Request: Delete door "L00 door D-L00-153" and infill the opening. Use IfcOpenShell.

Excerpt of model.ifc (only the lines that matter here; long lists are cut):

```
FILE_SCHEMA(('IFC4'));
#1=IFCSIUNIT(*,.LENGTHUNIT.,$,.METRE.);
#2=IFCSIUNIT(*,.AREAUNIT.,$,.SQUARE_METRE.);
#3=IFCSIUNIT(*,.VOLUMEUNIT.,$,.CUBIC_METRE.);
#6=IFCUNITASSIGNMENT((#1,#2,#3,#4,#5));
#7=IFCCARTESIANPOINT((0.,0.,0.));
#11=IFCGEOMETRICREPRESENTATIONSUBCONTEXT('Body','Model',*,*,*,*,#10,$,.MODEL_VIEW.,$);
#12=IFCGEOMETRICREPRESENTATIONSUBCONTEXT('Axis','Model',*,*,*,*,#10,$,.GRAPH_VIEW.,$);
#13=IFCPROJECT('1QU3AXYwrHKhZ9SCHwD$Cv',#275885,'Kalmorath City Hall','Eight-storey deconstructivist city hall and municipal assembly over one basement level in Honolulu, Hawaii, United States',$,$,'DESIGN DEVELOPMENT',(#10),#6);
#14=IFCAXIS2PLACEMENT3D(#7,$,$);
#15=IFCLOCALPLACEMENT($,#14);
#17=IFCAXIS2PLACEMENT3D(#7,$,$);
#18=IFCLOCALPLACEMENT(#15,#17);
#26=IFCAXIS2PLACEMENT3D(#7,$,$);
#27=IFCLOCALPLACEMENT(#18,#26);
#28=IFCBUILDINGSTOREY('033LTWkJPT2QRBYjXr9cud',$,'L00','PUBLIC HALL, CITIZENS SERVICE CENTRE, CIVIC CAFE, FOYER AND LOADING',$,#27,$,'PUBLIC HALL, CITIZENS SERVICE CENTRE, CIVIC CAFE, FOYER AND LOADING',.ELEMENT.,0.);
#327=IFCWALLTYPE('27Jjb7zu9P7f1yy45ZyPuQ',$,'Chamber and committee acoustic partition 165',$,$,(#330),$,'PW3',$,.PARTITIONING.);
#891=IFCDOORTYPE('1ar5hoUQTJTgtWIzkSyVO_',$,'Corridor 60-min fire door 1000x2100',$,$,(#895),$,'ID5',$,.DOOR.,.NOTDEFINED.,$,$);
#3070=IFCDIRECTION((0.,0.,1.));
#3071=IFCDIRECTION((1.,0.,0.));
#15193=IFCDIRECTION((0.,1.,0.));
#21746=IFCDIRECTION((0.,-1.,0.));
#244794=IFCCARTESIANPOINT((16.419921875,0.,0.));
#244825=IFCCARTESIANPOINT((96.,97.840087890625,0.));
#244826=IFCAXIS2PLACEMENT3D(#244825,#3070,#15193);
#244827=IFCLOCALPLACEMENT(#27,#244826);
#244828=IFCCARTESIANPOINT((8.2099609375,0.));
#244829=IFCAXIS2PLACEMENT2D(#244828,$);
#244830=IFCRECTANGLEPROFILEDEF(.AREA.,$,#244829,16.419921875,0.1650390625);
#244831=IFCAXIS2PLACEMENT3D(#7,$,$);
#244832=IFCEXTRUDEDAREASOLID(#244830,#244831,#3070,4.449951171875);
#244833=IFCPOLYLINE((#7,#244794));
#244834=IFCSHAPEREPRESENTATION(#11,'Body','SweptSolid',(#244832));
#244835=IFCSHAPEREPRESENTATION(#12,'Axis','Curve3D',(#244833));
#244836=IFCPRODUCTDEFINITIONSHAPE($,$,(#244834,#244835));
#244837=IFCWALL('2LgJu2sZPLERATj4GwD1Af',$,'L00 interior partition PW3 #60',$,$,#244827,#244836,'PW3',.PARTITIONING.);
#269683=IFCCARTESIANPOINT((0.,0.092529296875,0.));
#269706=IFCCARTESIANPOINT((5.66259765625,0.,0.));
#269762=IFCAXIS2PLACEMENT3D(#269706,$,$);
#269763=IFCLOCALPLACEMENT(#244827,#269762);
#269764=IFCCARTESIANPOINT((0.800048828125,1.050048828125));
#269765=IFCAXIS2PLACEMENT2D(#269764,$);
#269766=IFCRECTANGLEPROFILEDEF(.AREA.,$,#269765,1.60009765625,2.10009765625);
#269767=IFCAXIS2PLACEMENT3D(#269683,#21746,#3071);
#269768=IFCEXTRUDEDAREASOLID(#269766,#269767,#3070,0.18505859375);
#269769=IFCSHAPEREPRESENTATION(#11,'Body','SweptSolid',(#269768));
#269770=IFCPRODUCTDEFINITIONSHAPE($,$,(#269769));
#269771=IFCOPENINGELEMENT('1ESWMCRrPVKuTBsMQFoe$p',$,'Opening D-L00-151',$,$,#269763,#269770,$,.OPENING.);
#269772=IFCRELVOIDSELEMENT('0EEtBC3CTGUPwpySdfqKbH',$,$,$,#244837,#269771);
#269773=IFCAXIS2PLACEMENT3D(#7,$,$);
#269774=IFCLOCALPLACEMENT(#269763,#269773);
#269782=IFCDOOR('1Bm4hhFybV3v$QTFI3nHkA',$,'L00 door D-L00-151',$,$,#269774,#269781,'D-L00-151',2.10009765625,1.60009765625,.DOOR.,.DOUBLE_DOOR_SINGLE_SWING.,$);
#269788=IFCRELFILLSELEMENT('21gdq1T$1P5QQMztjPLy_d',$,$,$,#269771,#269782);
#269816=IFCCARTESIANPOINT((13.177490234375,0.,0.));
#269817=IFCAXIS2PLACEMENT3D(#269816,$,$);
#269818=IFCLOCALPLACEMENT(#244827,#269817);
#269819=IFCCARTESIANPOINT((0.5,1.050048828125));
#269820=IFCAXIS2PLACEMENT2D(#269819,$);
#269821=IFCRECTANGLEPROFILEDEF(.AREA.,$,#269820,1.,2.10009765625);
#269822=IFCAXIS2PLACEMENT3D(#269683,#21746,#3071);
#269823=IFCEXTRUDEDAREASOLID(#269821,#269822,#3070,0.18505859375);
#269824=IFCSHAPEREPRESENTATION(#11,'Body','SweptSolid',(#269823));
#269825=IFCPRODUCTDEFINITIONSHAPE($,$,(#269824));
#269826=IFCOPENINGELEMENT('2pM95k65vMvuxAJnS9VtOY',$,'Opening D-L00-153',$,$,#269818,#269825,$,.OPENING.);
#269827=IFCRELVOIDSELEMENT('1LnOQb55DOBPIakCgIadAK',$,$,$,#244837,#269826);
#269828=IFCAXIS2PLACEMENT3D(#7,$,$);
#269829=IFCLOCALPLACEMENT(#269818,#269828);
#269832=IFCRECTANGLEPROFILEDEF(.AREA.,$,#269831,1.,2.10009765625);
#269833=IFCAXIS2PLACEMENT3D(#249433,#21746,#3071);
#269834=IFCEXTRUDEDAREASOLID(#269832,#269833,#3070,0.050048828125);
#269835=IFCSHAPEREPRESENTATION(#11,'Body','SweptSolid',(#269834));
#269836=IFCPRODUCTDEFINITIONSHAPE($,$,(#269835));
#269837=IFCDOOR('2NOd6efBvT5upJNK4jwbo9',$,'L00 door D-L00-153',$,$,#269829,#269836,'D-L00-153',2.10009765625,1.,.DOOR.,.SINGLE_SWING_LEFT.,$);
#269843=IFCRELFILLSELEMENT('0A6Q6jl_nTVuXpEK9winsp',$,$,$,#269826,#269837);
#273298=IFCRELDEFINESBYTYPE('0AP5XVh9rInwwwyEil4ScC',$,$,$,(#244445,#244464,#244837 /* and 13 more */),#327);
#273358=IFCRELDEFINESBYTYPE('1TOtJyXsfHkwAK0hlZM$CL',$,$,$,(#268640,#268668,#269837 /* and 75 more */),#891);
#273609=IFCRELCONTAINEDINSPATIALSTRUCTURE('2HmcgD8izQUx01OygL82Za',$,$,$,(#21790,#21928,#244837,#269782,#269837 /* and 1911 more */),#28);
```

```python
import ifcopenshell
import ifcopenshell.api.feature
import ifcopenshell.api.root
import ifcopenshell.geom
import ifcopenshell.util.shape

model = ifcopenshell.open("model.ifc")
settings = ifcopenshell.geom.settings()


def volume(element):
    """Net volume in cubic metres, openings subtracted."""
    shape = ifcopenshell.geom.create_shape(settings, element)
    return ifcopenshell.util.shape.get_volume(shape.geometry)


door = model.by_guid("2NOd6efBvT5upJNK4jwbo9")
opening = door.FillsVoids[0].RelatingOpeningElement
wall = opening.VoidsElements[0].RelatingBuildingElement
before = volume(wall)

ifcopenshell.api.root.remove_product(model, product=door)
ifcopenshell.api.feature.remove_feature(model, feature=opening)

after = volume(wall)

print(f"wall volume {before:.3f} -> {after:.3f} m3")

model.write("model_v2.ifc")
```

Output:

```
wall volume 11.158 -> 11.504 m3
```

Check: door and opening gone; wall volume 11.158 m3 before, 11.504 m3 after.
